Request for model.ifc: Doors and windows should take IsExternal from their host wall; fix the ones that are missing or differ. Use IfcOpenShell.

First a look at what the model holds.

```python
import ifcopenshell
import ifcopenshell.util.element

model = ifcopenshell.open("model.ifc")
print(model.schema)
seen = {}
for e in model.by_type("IfcDoor") + model.by_type("IfcWindow"):
    if not e.FillsVoids:
        continue
    host = e.FillsVoids[0].RelatingOpeningElement.VoidsElements[0].RelatingBuildingElement
    own = ifcopenshell.util.element.get_pset(e, f"Pset_{e.is_a()[3:].removesuffix('StandardCase')}Common", "IsExternal")
    wall = ifcopenshell.util.element.get_pset(host, "Pset_WallCommon", "IsExternal")
    seen[e.is_a(), own, wall] = seen.get((e.is_a(), own, wall), 0) + 1
for (cls, own, wall), count in sorted(seen.items(), key=str):
    print(count, cls, "IsExternal:", own, "| host wall:", wall)
```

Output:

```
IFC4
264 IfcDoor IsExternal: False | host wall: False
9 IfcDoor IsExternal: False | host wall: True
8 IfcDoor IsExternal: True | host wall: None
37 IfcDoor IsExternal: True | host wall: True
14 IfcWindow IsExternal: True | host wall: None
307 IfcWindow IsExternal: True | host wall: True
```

```python
import ifcopenshell
import ifcopenshell.api.pset
import ifcopenshell.util.element

model = ifcopenshell.open("model.ifc")

count = 0
for ifc_class, pset_name in (("IfcDoor", "Pset_DoorCommon"), ("IfcWindow", "Pset_WindowCommon")):
    for e in model.by_type(ifc_class):
        if not e.FillsVoids:
            continue
        host = e.FillsVoids[0].RelatingOpeningElement.VoidsElements[0].RelatingBuildingElement
        external = ifcopenshell.util.element.get_pset(host, "Pset_WallCommon", "IsExternal")
        if external is None or ifcopenshell.util.element.get_pset(e, pset_name, "IsExternal") == external:
            continue
        pset = ifcopenshell.api.pset.add_pset(model, product=e, name=pset_name)
        ifcopenshell.api.pset.edit_pset(model, pset=pset, properties={"IsExternal": external})
        count += 1

print(count, "updated")

model.write("model_v2.ifc")
```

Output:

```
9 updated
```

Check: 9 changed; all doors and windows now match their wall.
